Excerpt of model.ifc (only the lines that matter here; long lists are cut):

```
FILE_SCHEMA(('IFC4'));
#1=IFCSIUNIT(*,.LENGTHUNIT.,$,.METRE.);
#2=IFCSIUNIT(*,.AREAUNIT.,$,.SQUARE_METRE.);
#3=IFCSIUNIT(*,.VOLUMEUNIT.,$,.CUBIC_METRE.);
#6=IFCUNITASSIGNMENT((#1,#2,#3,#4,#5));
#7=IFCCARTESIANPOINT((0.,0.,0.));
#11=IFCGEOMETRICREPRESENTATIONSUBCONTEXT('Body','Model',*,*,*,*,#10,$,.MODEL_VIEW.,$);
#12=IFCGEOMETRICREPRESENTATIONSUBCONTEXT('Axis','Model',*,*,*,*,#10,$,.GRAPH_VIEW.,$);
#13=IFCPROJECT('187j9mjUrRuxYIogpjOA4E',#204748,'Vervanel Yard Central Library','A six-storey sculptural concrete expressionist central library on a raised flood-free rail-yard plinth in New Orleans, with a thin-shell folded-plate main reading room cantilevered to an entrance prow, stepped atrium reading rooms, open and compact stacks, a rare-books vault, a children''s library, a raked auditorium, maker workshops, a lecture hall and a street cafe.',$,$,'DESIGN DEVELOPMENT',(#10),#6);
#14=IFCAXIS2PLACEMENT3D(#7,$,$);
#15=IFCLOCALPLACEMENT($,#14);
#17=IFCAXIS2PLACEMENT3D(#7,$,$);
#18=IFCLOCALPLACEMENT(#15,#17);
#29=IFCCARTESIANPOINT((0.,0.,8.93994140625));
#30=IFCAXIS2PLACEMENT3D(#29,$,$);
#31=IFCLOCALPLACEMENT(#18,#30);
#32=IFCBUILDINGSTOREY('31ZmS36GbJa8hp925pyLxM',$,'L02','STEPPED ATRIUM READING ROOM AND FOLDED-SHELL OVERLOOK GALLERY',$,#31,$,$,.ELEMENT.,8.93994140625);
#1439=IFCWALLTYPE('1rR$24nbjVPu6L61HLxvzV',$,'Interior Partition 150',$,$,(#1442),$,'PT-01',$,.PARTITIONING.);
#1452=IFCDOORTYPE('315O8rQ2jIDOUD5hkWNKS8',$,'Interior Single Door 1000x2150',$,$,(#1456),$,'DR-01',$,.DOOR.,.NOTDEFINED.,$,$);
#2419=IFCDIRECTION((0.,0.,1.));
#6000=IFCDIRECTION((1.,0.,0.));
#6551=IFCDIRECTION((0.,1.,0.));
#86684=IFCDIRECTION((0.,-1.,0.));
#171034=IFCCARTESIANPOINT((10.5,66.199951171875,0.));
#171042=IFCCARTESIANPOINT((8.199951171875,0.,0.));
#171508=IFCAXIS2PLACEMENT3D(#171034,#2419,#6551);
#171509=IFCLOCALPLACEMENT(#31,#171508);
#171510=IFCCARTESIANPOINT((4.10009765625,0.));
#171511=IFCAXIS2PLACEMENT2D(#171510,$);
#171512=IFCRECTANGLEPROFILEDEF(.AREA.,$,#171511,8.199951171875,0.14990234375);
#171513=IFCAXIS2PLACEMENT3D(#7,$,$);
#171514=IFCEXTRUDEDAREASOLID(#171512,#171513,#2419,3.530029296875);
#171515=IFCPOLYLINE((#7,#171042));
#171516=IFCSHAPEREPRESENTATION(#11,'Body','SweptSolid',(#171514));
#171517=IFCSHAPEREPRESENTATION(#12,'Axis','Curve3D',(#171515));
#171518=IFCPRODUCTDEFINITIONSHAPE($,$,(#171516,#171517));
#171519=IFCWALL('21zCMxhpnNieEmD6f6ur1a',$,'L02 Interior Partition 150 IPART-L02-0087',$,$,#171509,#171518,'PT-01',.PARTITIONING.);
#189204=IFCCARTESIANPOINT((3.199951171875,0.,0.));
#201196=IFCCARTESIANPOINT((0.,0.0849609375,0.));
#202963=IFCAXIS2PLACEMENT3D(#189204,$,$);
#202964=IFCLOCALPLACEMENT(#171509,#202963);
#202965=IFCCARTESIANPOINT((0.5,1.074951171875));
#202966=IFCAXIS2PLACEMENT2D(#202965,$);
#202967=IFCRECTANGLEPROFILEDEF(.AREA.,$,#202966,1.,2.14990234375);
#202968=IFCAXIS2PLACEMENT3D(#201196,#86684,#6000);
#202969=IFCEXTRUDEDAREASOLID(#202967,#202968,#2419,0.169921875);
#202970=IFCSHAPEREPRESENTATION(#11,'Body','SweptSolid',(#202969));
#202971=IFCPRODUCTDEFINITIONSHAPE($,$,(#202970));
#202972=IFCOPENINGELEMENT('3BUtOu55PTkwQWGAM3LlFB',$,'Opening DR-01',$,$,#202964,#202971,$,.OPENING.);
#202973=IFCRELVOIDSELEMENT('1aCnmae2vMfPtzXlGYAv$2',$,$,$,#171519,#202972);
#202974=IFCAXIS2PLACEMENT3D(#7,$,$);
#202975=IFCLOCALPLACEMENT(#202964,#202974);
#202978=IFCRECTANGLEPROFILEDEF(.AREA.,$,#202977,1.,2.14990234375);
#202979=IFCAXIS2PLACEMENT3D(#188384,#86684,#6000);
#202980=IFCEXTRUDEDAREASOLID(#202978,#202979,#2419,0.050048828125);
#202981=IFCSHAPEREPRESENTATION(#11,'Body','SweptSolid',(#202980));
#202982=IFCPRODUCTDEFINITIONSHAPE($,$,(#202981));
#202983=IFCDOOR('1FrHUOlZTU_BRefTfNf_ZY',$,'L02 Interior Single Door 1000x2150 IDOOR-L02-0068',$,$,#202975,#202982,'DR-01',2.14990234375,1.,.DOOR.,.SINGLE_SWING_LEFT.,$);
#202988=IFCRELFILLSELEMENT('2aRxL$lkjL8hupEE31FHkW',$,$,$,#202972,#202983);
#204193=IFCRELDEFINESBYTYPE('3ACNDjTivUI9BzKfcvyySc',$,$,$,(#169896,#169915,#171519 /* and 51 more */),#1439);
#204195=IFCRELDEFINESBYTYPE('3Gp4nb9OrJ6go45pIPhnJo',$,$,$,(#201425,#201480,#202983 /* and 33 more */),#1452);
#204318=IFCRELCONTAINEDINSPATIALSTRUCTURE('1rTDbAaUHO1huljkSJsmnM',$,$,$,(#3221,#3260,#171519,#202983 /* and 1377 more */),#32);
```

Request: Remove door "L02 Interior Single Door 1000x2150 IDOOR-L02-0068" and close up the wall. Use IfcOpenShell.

```python
import ifcopenshell
import ifcopenshell.api.feature
import ifcopenshell.api.root
import ifcopenshell.geom
import ifcopenshell.util.shape

model = ifcopenshell.open("model.ifc")
settings = ifcopenshell.geom.settings()


def volume(element):
    """Net volume in cubic metres, openings subtracted."""
    shape = ifcopenshell.geom.create_shape(settings, element)
    return ifcopenshell.util.shape.get_volume(shape.geometry)


door = model.by_guid("1FrHUOlZTU_BRefTfNf_ZY")
opening = door.FillsVoids[0].RelatingOpeningElement
wall = opening.VoidsElements[0].RelatingBuildingElement
before = volume(wall)

ifcopenshell.api.root.remove_product(model, product=door)
ifcopenshell.api.feature.remove_feature(model, feature=opening)

after = volume(wall)

print(f"wall volume {before:.3f} -> {after:.3f} m3")

model.write("model-out.ifc")
```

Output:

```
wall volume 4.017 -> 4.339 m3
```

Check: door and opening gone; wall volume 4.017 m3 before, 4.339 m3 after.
